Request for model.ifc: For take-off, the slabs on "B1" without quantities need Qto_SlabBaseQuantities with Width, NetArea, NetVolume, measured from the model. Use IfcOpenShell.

First a look at what the model holds.

```python
import ifcopenshell
import ifcopenshell.util.element
import ifcopenshell.util.unit

model = ifcopenshell.open("model.ifc")
print(model.schema)
for unit_type in ("LENGTHUNIT", "AREAUNIT", "VOLUMEUNIT"):
    print(unit_type, ifcopenshell.util.unit.calculate_unit_scale(model, unit_type))
storey = next(s for s in model.by_type("IfcBuildingStorey") if s.Name == "B1")
slabs = [e for e in ifcopenshell.util.element.get_decomposition(storey) if e.is_a("IfcSlab")]
for e in sorted(slabs, key=lambda e: e.id()):
    print(e.id(), e.is_a(), e.Name, list(ifcopenshell.util.element.get_psets(e, qtos_only=True)), sep=" | ")
```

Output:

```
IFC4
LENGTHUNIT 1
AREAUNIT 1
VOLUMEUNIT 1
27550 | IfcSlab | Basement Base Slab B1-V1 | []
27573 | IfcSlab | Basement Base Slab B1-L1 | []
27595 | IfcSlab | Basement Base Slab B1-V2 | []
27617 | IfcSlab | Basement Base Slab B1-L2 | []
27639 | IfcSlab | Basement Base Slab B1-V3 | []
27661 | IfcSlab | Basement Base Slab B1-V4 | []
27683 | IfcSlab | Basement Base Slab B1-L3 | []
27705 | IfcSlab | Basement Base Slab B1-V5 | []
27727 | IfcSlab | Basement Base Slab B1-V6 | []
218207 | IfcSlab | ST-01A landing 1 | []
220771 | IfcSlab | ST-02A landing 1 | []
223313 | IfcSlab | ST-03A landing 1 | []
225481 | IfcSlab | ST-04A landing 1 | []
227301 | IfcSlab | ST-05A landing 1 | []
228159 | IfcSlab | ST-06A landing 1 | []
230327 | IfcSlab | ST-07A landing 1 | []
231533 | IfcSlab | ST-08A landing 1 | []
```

```python
import ifcopenshell
import ifcopenshell.api.pset
import ifcopenshell.geom
import ifcopenshell.util.element
import ifcopenshell.util.shape
import ifcopenshell.util.unit

model = ifcopenshell.open("model.ifc")
unit_scale = ifcopenshell.util.unit.calculate_unit_scale(model)
area_scale = ifcopenshell.util.unit.calculate_unit_scale(model, "AREAUNIT")
volume_scale = ifcopenshell.util.unit.calculate_unit_scale(model, "VOLUMEUNIT")
settings = ifcopenshell.geom.settings()

storey = next(s for s in model.by_type("IfcBuildingStorey") if s.Name == "B1")
slabs = [e for e in ifcopenshell.util.element.get_decomposition(storey) if e.is_a("IfcSlab")]

for e in sorted(slabs, key=lambda e: e.id()):
    if ifcopenshell.util.element.get_psets(e, qtos_only=True, should_inherit=False):
        continue
    # Geometry comes back in metres, in the element's own axes.
    shape = ifcopenshell.geom.create_shape(settings, e)
    values = {
        "Width": ifcopenshell.util.shape.get_z(shape.geometry) / unit_scale,
        "NetArea": ifcopenshell.util.shape.get_footprint_area(shape.geometry) / area_scale,
        "NetVolume": ifcopenshell.util.shape.get_volume(shape.geometry) / volume_scale,
    }
    qto = ifcopenshell.api.pset.add_qto(model, product=e, name="Qto_SlabBaseQuantities")
    ifcopenshell.api.pset.edit_qto(model, qto=qto, properties=values)
    print(e.id(), {k: round(v, 3) for k, v in values.items()})

model.write("model_edited.ifc")
```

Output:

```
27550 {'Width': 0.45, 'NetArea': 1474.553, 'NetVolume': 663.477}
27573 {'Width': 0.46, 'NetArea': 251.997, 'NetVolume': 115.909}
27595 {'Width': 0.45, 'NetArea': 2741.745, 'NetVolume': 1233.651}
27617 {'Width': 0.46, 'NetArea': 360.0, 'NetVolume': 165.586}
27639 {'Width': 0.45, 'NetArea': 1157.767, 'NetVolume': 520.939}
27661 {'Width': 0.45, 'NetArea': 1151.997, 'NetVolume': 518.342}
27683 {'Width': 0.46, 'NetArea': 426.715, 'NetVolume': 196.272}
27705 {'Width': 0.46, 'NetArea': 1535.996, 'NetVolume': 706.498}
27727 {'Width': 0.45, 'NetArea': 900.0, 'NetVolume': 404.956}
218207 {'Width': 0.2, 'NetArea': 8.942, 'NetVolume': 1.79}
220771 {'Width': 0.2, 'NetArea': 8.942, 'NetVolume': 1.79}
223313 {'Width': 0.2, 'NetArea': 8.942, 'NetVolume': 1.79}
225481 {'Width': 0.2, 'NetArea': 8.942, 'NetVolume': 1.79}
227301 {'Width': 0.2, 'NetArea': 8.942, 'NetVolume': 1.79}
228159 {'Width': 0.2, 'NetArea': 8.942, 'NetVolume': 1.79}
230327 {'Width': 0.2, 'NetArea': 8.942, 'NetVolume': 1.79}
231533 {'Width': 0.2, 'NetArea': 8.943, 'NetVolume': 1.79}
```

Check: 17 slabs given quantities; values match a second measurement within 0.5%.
